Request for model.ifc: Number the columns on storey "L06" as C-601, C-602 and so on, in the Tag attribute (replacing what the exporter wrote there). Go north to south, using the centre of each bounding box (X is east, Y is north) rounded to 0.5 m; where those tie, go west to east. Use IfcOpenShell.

First a look at what the model holds.

```python
import ifcopenshell
import ifcopenshell.util.element
import ifcopenshell.util.placement

model = ifcopenshell.open("model.ifc")
print(model.schema)
storey = next(s for s in model.by_type("IfcBuildingStorey") if s.Name == "L06")
columns = [e for e in ifcopenshell.util.element.get_decomposition(storey) if e.is_a("IfcColumn")]
for e in sorted(columns, key=lambda e: e.id()):
    origin = ifcopenshell.util.placement.get_local_placement(e.ObjectPlacement)[:3, 3]
    print(e.id(), e.Tag, e.Name, origin.round(2) + 0.0, sep=" | ")
```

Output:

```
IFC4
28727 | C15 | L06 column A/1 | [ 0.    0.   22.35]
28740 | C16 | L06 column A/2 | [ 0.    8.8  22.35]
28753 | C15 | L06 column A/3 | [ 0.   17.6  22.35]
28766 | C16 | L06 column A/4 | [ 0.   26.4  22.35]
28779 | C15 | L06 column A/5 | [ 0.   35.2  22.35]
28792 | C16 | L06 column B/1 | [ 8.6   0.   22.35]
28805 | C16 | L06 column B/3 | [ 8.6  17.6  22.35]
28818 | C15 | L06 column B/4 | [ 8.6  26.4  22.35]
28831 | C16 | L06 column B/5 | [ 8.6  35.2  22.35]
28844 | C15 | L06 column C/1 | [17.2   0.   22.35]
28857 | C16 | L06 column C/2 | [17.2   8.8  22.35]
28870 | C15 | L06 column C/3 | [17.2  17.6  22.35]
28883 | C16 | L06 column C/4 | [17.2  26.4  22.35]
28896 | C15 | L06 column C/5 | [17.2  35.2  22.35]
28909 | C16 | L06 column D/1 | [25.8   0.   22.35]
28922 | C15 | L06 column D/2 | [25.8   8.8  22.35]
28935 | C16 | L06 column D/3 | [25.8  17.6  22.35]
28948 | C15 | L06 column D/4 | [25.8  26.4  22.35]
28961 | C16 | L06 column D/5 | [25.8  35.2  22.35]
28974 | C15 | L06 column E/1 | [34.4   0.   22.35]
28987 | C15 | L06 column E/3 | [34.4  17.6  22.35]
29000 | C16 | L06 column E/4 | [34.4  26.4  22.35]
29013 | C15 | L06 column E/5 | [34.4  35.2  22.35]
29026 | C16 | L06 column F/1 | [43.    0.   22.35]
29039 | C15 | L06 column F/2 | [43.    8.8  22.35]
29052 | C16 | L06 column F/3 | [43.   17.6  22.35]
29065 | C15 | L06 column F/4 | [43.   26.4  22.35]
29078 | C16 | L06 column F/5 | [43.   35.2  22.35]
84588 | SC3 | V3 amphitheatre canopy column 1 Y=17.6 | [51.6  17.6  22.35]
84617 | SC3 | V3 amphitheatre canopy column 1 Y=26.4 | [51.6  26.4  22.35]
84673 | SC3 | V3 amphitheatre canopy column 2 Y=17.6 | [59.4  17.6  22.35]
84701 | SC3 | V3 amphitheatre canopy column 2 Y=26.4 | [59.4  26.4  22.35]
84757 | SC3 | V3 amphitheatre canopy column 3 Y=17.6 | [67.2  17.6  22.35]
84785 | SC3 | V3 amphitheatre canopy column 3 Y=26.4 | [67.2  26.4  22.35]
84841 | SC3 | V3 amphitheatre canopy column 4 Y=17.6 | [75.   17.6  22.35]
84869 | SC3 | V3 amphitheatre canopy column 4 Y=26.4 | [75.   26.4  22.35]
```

```python
import ifcopenshell
import ifcopenshell.geom
import ifcopenshell.util.element
import ifcopenshell.util.shape

model = ifcopenshell.open("model.ifc")
settings = ifcopenshell.geom.settings()
settings.set("use-world-coords", True)


def centre(element):
    shape = ifcopenshell.geom.create_shape(settings, element)
    return ifcopenshell.util.shape.get_bbox_centroid(shape.geometry)


storey = next(s for s in model.by_type("IfcBuildingStorey") if s.Name == "L06")
columns = [e for e in ifcopenshell.util.element.get_decomposition(storey) if e.is_a("IfcColumn")]

# Insertion points can sit at a corner or the storey origin, so sort by the geometry (in metres).
centres = {e: centre(e) for e in columns}
columns.sort(key=lambda e: (-round(centres[e][1] / 0.5), centres[e][0]))

for i, e in enumerate(columns, start=1):
    number = f"C-6{i:02d}"
    e.Tag = number
    print(e.id(), number)

model.write("model_updated.ifc")
```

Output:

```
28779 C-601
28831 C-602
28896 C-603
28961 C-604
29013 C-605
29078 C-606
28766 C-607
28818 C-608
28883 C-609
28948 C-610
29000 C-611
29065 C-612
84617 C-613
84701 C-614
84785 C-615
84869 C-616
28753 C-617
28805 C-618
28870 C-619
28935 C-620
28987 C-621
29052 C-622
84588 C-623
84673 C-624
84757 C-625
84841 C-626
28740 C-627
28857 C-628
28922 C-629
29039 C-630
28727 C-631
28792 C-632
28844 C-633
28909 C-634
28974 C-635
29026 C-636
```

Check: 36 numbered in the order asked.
